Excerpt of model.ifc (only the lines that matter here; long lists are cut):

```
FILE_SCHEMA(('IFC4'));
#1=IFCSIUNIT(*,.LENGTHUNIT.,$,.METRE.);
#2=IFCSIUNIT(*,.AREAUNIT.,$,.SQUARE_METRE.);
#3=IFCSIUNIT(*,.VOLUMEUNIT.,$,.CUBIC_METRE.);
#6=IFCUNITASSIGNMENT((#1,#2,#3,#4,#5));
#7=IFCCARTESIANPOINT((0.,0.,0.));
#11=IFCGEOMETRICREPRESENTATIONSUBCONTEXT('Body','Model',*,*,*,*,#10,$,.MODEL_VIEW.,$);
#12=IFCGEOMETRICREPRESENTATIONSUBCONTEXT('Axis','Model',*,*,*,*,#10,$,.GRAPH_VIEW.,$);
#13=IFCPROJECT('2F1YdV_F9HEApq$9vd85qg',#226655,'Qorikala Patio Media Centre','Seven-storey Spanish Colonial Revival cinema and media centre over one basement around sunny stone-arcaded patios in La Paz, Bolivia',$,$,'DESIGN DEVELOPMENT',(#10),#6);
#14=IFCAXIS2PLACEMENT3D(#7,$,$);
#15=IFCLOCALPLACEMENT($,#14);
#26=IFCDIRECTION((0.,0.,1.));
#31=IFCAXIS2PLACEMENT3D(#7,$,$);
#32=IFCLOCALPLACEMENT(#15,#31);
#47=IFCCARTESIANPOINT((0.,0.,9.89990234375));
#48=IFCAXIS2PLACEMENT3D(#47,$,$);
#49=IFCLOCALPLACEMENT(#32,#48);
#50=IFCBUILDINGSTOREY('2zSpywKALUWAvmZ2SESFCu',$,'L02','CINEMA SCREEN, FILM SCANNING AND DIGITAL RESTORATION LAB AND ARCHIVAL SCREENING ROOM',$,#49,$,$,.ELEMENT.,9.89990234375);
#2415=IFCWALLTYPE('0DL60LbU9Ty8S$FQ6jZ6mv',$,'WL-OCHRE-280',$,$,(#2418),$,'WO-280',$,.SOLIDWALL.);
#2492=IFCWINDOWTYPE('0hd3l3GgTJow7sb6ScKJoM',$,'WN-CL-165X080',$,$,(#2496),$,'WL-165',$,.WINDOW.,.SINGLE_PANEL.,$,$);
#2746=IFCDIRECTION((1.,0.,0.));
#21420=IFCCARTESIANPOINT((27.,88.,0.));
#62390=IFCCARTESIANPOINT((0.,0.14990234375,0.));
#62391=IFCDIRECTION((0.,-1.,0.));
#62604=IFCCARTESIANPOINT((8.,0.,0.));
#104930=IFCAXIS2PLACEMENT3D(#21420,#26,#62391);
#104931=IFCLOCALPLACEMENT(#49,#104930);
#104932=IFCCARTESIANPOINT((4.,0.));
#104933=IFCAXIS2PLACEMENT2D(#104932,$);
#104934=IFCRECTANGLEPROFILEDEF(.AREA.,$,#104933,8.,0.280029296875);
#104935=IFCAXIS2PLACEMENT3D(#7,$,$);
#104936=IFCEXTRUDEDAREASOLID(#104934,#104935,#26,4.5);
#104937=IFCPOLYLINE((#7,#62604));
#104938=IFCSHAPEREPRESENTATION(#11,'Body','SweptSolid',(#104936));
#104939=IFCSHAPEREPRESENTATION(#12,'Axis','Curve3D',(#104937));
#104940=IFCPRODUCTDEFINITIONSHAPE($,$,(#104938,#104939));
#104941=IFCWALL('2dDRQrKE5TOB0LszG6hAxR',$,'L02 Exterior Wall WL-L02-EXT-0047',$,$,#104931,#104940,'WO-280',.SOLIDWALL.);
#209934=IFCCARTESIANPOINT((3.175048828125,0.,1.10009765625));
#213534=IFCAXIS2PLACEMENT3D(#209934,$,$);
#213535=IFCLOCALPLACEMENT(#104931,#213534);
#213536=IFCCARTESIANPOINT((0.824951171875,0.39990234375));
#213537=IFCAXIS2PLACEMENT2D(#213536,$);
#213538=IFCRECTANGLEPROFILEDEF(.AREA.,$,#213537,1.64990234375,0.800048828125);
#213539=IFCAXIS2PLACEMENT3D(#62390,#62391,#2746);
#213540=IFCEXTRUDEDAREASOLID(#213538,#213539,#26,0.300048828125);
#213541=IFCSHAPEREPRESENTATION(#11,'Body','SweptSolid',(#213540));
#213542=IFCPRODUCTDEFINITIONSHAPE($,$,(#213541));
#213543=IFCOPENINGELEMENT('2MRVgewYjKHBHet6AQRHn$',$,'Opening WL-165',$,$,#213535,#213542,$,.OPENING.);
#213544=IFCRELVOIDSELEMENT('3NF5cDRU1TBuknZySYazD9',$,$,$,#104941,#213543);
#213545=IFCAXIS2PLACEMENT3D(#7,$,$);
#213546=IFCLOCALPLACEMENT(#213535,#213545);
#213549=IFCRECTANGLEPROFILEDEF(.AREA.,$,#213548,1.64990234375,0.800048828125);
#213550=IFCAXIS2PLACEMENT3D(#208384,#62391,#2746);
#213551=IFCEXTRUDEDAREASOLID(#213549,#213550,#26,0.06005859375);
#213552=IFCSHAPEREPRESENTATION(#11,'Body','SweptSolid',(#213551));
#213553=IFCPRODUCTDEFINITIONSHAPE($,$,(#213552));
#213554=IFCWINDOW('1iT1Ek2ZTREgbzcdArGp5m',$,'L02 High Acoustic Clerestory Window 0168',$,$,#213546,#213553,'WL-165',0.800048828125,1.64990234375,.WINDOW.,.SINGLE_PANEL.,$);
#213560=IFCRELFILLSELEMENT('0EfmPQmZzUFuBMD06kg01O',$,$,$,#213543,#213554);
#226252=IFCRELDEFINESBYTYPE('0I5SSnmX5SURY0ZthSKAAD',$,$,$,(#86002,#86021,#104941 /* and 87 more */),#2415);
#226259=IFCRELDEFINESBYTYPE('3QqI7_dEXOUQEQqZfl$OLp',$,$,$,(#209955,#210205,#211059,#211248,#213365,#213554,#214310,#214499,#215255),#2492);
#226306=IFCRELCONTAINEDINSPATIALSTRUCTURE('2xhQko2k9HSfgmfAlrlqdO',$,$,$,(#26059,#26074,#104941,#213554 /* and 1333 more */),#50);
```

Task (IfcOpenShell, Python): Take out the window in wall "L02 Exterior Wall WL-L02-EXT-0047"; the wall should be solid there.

```python
import ifcopenshell
import ifcopenshell.api.feature
import ifcopenshell.api.root
import ifcopenshell.geom
import ifcopenshell.util.shape

model = ifcopenshell.open("model.ifc")
settings = ifcopenshell.geom.settings()


def volume(element):
    """Net volume in cubic metres, openings subtracted."""
    shape = ifcopenshell.geom.create_shape(settings, element)
    return ifcopenshell.util.shape.get_volume(shape.geometry)


window = model.by_id(213554)
opening = window.FillsVoids[0].RelatingOpeningElement
wall = opening.VoidsElements[0].RelatingBuildingElement
before = volume(wall)

ifcopenshell.api.root.remove_product(model, product=window)
ifcopenshell.api.feature.remove_feature(model, feature=opening)

after = volume(wall)

print(f"wall volume {before:.3f} -> {after:.3f} m3")

model.write("model_v2.ifc")
```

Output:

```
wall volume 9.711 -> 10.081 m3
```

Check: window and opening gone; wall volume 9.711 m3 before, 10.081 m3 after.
